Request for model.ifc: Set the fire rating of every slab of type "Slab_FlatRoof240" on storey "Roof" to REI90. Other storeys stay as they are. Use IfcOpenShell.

First a look at what the model holds.

```python
import ifcopenshell
import ifcopenshell.util.element

model = ifcopenshell.open("model.ifc")
print(model.schema)
storey = next(s for s in model.by_type("IfcBuildingStorey") if s.Name == "Roof")
slabs = [e for e in ifcopenshell.util.element.get_decomposition(storey) if e.is_a("IfcSlab")]
seen = {}
for e in slabs:
    element_type = ifcopenshell.util.element.get_type(e)
    key = (element_type.Name if element_type != e and element_type else None, ifcopenshell.util.element.get_pset(e, "Pset_SlabCommon", "FireRating"))
    seen[key] = seen.get(key, 0) + 1
for (name, value), count in sorted(seen.items(), key=str):
    print(count, "x", name, "|", value)
```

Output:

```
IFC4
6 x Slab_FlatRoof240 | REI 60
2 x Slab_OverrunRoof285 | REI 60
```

```python
import ifcopenshell
import ifcopenshell.api.pset
import ifcopenshell.util.element

model = ifcopenshell.open("model.ifc")

storey = next(s for s in model.by_type("IfcBuildingStorey") if s.Name == "Roof")
slabs = [e for e in ifcopenshell.util.element.get_decomposition(storey) if e.is_a("IfcSlab")]

count = 0
for e in slabs:
    element_type = ifcopenshell.util.element.get_type(e)
    if element_type in (None, e) or element_type.Name != "Slab_FlatRoof240":
        continue
    # add_pset returns the element's existing set when there is one.
    pset = ifcopenshell.api.pset.add_pset(model, product=e, name="Pset_SlabCommon")
    ifcopenshell.api.pset.edit_pset(model, pset=pset, properties={"FireRating": "REI90"})
    count += 1

print(count, "slabs updated")

model.write("model-out.ifc")
```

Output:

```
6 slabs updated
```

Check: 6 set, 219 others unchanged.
